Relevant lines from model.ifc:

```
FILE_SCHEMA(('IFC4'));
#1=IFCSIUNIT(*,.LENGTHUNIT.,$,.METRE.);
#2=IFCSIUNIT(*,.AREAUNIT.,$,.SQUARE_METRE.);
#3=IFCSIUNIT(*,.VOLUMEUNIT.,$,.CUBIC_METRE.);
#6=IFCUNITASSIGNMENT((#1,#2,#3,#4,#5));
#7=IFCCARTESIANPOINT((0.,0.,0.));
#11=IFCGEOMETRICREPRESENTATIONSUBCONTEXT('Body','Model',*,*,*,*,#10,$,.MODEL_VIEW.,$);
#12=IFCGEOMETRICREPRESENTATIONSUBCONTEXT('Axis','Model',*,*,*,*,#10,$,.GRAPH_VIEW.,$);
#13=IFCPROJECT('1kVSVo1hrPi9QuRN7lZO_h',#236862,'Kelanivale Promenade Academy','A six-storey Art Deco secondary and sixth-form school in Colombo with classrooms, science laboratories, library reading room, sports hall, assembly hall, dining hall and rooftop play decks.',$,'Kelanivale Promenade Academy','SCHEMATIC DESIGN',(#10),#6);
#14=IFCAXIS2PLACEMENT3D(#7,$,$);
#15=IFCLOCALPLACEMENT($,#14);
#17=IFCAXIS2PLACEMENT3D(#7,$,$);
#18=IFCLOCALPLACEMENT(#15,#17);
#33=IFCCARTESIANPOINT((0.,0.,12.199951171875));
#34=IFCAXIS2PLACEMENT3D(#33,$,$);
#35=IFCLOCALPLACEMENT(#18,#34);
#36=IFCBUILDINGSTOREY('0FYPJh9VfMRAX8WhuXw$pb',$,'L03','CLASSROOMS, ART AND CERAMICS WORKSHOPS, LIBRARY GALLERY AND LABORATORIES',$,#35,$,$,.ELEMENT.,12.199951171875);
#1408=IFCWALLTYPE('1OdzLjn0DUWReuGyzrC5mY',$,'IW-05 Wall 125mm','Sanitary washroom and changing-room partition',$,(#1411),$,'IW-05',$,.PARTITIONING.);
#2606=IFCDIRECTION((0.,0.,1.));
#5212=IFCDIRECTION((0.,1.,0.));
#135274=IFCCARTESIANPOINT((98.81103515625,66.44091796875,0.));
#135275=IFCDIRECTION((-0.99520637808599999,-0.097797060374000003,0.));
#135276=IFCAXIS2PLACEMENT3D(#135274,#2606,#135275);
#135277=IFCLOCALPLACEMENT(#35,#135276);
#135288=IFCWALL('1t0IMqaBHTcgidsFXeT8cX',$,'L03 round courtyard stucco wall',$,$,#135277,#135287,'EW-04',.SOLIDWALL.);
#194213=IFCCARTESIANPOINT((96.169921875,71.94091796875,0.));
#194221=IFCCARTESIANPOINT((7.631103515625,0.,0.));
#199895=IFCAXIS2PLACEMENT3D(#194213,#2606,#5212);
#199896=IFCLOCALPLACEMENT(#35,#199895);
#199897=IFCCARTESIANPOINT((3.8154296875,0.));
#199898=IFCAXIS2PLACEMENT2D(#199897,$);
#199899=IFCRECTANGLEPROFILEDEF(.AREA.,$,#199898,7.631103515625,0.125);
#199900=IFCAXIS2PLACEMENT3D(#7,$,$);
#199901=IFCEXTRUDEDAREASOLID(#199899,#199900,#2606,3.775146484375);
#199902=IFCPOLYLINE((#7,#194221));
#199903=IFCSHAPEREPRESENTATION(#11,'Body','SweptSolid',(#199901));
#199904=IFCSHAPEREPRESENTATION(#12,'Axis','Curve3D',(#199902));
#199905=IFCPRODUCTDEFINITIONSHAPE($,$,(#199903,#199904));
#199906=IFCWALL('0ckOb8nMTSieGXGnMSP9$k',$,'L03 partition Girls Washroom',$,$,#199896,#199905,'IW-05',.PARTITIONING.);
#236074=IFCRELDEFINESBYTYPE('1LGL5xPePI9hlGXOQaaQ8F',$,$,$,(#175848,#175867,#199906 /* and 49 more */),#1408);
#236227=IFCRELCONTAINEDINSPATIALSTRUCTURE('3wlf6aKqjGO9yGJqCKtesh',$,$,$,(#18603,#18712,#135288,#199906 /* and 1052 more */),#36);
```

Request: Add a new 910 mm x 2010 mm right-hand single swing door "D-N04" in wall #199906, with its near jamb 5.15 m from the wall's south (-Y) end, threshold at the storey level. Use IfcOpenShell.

```python
import numpy as np
import ifcopenshell
import ifcopenshell.api.feature
import ifcopenshell.api.geometry
import ifcopenshell.api.root
import ifcopenshell.api.spatial
import ifcopenshell.geom
import ifcopenshell.util.element
import ifcopenshell.util.placement
import ifcopenshell.util.representation
import ifcopenshell.util.shape
import ifcopenshell.util.unit

model = ifcopenshell.open("model.ifc")
unit_scale = ifcopenshell.util.unit.calculate_unit_scale(model)
settings = ifcopenshell.geom.settings()


def volume(element):
    """Net volume in cubic metres, openings subtracted."""
    shape = ifcopenshell.geom.create_shape(settings, element)
    return ifcopenshell.util.shape.get_volume(shape.geometry)


wall = model.by_guid("0ckOb8nMTSieGXGnMSP9$k")
storey = ifcopenshell.util.element.get_container(wall, ifc_class="IfcBuildingStorey")
context = ifcopenshell.util.representation.get_context(model, "Model", "Body", "MODEL_VIEW")
before = volume(wall)

width, height, from_end, sill = 0.91, 2.01, 5.15, 0.0  # metres

# The wall runs along its own X axis, and the end named is its -X end.
wall_shape = ifcopenshell.geom.create_shape(settings, wall)
x, y, z = ifcopenshell.util.shape.get_vertices(wall_shape.geometry).T
start = x.min() + from_end
face, thickness = float(y.min()), float(y.max() - y.min())
wall_matrix = ifcopenshell.util.placement.get_local_placement(wall.ObjectPlacement)
level = ifcopenshell.util.placement.get_local_placement(storey.ObjectPlacement)[2, 3]


def in_wall(x, y):
    """Placement at x, y metres in the wall's axes, at sill height."""
    matrix = wall_matrix.copy()
    matrix[:, 3] = wall_matrix @ np.array([x / unit_scale, y / unit_scale, 0.0, 1.0])
    matrix[2, 3] = level + sill / unit_scale
    return matrix


# Opening: a box that overshoots both wall faces by 50 mm.
opening = ifcopenshell.api.root.create_entity(model, ifc_class="IfcOpeningElement", predefined_type="OPENING")
box = ifcopenshell.api.geometry.add_wall_representation(
    model, context=context, length=width, height=height, thickness=thickness + 0.1
)
ifcopenshell.api.geometry.assign_representation(model, product=opening, representation=box)
ifcopenshell.api.geometry.edit_object_placement(model, product=opening, matrix=in_wall(start, face - 0.05), is_si=False)
ifcopenshell.api.feature.add_feature(model, feature=opening, element=wall)

door = ifcopenshell.api.root.create_entity(model, ifc_class="IfcDoor", name="D-N04", predefined_type="DOOR")
door.OverallWidth, door.OverallHeight = width / unit_scale, height / unit_scale
door.OperationType = "SINGLE_SWING_RIGHT"
body = ifcopenshell.api.geometry.add_door_representation(
    model,
    context=context,
    overall_width=door.OverallWidth,
    overall_height=door.OverallHeight,
    operation_type="SINGLE_SWING_RIGHT",
    lining_properties={"LiningDepth": thickness / unit_scale, "ThresholdDepth": thickness / unit_scale},
)
ifcopenshell.api.geometry.assign_representation(model, product=door, representation=body)
ifcopenshell.api.spatial.assign_container(model, products=[door], relating_structure=storey)
ifcopenshell.api.feature.add_filling(model, opening=opening, element=door)

# The lining spans the wall, so the door starts at the wall face.
ifcopenshell.api.geometry.edit_object_placement(model, product=door, matrix=in_wall(start, face), is_si=False)

after = volume(wall)

print(f"wall volume {before:.3f} -> {after:.3f} m3")

model.write("model_v2.ifc")
```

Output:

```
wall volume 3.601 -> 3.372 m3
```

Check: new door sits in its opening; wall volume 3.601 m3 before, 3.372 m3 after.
